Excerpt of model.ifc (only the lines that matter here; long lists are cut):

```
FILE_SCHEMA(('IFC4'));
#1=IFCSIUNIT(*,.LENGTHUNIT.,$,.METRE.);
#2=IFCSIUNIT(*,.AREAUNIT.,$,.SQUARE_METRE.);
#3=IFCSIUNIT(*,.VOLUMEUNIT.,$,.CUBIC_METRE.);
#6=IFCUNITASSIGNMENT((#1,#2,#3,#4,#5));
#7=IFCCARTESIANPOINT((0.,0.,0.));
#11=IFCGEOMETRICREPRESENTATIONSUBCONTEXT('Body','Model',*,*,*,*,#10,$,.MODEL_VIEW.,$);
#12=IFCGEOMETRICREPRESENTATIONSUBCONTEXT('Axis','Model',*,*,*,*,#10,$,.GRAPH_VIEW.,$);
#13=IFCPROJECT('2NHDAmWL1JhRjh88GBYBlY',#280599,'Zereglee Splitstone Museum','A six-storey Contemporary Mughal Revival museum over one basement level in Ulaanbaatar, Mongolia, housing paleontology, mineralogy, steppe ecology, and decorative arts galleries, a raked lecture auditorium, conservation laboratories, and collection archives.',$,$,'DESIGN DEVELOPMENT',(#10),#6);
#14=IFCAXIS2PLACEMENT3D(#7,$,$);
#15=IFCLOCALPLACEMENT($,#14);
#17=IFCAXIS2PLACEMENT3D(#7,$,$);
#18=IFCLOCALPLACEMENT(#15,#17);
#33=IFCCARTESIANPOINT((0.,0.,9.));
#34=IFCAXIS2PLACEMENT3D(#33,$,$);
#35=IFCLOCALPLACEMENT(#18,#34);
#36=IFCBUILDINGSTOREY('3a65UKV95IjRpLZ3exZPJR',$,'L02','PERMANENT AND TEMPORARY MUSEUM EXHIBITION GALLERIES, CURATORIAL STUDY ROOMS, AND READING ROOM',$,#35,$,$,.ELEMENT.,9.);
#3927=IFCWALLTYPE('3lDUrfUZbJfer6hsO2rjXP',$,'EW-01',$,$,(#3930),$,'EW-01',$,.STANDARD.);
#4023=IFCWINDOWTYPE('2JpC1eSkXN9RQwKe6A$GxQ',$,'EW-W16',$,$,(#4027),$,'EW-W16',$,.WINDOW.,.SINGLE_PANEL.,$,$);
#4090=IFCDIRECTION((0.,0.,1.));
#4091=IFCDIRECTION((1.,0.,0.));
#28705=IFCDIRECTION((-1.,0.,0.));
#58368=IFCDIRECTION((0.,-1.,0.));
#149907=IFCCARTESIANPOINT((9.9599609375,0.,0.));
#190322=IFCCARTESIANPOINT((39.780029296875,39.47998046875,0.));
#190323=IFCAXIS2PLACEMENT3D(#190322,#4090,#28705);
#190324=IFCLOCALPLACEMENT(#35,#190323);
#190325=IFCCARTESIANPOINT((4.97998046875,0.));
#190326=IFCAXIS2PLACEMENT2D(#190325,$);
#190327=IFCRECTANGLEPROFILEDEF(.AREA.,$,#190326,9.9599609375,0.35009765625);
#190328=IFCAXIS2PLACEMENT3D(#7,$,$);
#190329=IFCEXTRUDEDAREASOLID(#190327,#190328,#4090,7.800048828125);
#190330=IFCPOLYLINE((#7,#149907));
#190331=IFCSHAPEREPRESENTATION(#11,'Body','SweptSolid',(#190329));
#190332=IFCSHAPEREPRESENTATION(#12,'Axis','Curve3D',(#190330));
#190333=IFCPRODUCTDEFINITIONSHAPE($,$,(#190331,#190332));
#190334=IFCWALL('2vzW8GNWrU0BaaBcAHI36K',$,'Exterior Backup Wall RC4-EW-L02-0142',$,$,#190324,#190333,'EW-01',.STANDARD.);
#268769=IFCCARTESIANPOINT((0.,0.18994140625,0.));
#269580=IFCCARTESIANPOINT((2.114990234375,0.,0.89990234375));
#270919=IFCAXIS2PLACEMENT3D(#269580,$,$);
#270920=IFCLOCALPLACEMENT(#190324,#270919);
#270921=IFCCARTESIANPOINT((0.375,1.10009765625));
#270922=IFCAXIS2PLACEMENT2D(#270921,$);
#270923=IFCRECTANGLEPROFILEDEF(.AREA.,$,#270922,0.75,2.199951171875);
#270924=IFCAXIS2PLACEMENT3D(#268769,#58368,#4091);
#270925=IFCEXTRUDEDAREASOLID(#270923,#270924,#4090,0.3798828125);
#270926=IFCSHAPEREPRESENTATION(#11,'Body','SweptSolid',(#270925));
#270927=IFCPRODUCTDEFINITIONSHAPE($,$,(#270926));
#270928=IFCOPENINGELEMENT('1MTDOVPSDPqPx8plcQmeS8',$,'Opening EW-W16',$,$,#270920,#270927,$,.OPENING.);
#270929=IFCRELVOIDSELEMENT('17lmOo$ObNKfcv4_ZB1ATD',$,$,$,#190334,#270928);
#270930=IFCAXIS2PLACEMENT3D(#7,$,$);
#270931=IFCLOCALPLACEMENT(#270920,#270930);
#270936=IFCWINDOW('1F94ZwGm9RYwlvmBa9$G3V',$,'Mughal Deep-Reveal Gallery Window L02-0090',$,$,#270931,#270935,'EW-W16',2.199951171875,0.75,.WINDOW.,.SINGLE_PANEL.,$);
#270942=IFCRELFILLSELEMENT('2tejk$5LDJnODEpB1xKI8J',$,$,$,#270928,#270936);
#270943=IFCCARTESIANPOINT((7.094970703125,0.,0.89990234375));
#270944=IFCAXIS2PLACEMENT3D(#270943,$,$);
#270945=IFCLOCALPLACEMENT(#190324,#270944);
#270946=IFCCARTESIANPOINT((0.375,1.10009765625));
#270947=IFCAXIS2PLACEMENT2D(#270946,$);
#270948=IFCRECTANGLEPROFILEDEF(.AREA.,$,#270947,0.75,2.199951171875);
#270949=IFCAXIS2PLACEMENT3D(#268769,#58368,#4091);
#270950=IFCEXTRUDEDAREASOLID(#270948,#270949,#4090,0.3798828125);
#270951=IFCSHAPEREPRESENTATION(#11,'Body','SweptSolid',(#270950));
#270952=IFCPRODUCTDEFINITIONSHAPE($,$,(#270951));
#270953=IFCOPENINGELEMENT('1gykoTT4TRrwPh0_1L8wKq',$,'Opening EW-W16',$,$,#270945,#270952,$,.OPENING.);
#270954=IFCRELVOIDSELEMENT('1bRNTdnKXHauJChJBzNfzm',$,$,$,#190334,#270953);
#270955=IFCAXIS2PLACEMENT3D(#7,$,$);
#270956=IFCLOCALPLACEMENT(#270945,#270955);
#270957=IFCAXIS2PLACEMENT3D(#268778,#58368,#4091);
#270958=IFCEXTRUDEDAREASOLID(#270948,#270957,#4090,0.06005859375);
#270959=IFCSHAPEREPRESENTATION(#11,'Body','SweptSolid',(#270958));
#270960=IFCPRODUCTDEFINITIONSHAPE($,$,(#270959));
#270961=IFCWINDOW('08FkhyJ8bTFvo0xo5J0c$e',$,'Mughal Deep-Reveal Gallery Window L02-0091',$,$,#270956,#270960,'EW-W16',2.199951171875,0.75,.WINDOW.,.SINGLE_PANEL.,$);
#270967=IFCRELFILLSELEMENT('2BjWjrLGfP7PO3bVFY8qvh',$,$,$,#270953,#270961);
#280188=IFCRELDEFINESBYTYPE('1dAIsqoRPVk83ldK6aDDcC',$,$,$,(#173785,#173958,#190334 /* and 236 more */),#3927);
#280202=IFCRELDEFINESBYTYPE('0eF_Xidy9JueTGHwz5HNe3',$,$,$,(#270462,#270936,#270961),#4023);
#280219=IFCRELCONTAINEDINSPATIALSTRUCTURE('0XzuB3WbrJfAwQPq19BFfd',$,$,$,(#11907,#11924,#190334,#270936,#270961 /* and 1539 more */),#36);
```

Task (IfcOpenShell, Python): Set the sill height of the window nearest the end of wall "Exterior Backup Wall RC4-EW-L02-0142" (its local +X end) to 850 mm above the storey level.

```python
import numpy as np
import ifcopenshell
import ifcopenshell.api.geometry
import ifcopenshell.geom
import ifcopenshell.util.element
import ifcopenshell.util.placement
import ifcopenshell.util.shape
import ifcopenshell.util.unit

model = ifcopenshell.open("model.ifc")
unit_scale = ifcopenshell.util.unit.calculate_unit_scale(model)

window = model.by_guid("08FkhyJ8bTFvo0xo5J0c$e")
opening = window.FillsVoids[0].RelatingOpeningElement
storey = ifcopenshell.util.element.get_container(window, ifc_class="IfcBuildingStorey")
level = ifcopenshell.util.placement.get_local_placement(storey.ObjectPlacement)[2, 3]

# The opening's origin need not be at the sill, so measure its lowest point.
shape = ifcopenshell.geom.create_shape(ifcopenshell.geom.settings(), opening)
bottom = ifcopenshell.util.shape.get_shape_bottom_elevation(shape, shape.geometry) / unit_scale
dz = level + 0.85 - bottom

shift = np.array([0.0, 0.0, dz])
# The window is placed relative to its opening, so it follows when the opening moves.
matrix = ifcopenshell.util.placement.get_local_placement(opening.ObjectPlacement)
matrix[:3, 3] += shift
ifcopenshell.api.geometry.edit_object_placement(
    model, product=opening, matrix=matrix, is_si=False, should_transform_children=True
)

print(f"moved by {dz * unit_scale:+.3f} m")

model.write("model_updated.ifc")
```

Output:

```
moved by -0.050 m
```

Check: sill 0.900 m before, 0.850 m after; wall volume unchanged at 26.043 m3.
